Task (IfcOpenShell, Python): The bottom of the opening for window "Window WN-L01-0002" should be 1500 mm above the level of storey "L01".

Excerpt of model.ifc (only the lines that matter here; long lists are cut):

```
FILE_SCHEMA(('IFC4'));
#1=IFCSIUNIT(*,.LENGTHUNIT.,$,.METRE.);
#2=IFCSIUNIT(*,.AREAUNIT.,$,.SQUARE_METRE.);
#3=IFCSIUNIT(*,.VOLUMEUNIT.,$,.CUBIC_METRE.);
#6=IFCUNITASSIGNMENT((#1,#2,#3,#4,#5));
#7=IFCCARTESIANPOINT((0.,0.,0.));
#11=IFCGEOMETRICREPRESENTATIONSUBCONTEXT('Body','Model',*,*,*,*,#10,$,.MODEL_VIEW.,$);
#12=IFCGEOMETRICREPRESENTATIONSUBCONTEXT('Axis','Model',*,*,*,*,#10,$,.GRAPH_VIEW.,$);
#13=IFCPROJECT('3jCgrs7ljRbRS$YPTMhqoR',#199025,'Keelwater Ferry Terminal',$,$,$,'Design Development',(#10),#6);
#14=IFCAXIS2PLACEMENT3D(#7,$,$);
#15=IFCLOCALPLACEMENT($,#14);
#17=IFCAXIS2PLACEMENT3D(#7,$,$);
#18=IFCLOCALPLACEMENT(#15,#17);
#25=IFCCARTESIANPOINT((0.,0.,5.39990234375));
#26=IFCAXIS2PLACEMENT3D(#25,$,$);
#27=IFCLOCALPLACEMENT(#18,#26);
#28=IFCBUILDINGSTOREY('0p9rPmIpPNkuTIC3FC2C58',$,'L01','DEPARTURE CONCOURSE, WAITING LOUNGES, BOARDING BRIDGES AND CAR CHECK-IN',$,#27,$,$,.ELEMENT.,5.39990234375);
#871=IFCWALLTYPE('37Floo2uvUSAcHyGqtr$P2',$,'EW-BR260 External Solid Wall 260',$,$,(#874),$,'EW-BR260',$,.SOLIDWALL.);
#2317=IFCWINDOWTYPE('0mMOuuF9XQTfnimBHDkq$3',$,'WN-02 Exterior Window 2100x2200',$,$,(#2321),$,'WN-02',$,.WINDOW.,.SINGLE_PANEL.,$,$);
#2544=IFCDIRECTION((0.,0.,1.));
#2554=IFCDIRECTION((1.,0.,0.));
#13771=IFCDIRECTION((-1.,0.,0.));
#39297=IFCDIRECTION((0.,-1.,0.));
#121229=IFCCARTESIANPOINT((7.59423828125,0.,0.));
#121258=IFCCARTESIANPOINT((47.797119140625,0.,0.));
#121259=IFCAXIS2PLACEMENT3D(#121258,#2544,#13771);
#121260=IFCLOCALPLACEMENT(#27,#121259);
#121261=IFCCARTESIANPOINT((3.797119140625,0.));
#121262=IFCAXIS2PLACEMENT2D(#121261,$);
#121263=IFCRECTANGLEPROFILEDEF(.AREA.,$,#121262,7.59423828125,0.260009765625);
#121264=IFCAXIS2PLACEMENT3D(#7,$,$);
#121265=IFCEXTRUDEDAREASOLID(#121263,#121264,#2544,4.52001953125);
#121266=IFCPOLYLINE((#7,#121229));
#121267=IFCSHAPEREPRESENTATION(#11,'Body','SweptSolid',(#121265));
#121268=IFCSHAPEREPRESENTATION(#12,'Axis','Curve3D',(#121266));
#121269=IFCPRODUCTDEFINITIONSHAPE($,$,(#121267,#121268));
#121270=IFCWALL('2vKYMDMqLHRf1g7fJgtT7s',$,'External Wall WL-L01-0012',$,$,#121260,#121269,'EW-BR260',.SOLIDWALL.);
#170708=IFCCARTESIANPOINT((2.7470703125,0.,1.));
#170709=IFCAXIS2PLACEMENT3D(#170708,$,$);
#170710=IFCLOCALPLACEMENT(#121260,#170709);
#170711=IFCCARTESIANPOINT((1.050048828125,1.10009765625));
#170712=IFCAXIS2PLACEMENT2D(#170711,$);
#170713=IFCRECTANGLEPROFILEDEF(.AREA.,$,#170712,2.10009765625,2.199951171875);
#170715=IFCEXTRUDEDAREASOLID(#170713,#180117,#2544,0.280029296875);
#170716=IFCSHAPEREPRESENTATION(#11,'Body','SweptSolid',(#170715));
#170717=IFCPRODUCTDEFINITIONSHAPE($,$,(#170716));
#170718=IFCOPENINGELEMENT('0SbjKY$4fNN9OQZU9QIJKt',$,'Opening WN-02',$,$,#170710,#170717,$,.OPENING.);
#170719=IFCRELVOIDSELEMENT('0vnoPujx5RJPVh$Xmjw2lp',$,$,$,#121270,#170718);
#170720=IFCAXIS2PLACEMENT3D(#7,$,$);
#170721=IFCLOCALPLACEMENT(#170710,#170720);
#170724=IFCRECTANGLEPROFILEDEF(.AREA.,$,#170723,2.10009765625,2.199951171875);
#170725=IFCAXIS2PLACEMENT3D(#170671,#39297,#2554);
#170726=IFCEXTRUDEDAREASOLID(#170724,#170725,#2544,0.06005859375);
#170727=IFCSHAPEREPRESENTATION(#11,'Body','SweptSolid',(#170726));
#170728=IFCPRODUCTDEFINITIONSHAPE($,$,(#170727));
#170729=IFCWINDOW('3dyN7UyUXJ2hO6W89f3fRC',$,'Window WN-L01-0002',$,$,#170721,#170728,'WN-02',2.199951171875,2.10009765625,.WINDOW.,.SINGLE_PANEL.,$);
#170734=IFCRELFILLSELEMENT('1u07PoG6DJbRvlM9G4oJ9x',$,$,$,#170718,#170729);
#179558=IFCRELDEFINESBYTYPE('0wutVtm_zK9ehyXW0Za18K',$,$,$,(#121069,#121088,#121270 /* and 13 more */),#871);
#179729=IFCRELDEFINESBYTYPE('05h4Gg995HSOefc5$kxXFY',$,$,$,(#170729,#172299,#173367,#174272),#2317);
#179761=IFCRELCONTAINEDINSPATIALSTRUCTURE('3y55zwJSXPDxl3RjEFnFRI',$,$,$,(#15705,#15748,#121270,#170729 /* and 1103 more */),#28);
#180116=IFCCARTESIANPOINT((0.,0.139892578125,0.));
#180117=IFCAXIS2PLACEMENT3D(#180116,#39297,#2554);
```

```python
import numpy as np
import ifcopenshell
import ifcopenshell.api.geometry
import ifcopenshell.geom
import ifcopenshell.util.element
import ifcopenshell.util.placement
import ifcopenshell.util.shape
import ifcopenshell.util.unit

model = ifcopenshell.open("model.ifc")
unit_scale = ifcopenshell.util.unit.calculate_unit_scale(model)

window = model.by_guid("3dyN7UyUXJ2hO6W89f3fRC")
opening = window.FillsVoids[0].RelatingOpeningElement
storey = ifcopenshell.util.element.get_container(window, ifc_class="IfcBuildingStorey")
level = ifcopenshell.util.placement.get_local_placement(storey.ObjectPlacement)[2, 3]

# The opening's origin need not be at the sill, so measure its lowest point.
shape = ifcopenshell.geom.create_shape(ifcopenshell.geom.settings(), opening)
bottom = ifcopenshell.util.shape.get_shape_bottom_elevation(shape, shape.geometry) / unit_scale
dz = level + 1.5 - bottom

shift = np.array([0.0, 0.0, dz])
# The window is placed relative to its opening, so it follows when the opening moves.
matrix = ifcopenshell.util.placement.get_local_placement(opening.ObjectPlacement)
matrix[:3, 3] += shift
ifcopenshell.api.geometry.edit_object_placement(
    model, product=opening, matrix=matrix, is_si=False, should_transform_children=True
)

print(f"moved by {dz * unit_scale:+.3f} m")

model.write("model_edited.ifc")
```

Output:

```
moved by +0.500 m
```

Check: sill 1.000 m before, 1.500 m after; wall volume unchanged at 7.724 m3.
